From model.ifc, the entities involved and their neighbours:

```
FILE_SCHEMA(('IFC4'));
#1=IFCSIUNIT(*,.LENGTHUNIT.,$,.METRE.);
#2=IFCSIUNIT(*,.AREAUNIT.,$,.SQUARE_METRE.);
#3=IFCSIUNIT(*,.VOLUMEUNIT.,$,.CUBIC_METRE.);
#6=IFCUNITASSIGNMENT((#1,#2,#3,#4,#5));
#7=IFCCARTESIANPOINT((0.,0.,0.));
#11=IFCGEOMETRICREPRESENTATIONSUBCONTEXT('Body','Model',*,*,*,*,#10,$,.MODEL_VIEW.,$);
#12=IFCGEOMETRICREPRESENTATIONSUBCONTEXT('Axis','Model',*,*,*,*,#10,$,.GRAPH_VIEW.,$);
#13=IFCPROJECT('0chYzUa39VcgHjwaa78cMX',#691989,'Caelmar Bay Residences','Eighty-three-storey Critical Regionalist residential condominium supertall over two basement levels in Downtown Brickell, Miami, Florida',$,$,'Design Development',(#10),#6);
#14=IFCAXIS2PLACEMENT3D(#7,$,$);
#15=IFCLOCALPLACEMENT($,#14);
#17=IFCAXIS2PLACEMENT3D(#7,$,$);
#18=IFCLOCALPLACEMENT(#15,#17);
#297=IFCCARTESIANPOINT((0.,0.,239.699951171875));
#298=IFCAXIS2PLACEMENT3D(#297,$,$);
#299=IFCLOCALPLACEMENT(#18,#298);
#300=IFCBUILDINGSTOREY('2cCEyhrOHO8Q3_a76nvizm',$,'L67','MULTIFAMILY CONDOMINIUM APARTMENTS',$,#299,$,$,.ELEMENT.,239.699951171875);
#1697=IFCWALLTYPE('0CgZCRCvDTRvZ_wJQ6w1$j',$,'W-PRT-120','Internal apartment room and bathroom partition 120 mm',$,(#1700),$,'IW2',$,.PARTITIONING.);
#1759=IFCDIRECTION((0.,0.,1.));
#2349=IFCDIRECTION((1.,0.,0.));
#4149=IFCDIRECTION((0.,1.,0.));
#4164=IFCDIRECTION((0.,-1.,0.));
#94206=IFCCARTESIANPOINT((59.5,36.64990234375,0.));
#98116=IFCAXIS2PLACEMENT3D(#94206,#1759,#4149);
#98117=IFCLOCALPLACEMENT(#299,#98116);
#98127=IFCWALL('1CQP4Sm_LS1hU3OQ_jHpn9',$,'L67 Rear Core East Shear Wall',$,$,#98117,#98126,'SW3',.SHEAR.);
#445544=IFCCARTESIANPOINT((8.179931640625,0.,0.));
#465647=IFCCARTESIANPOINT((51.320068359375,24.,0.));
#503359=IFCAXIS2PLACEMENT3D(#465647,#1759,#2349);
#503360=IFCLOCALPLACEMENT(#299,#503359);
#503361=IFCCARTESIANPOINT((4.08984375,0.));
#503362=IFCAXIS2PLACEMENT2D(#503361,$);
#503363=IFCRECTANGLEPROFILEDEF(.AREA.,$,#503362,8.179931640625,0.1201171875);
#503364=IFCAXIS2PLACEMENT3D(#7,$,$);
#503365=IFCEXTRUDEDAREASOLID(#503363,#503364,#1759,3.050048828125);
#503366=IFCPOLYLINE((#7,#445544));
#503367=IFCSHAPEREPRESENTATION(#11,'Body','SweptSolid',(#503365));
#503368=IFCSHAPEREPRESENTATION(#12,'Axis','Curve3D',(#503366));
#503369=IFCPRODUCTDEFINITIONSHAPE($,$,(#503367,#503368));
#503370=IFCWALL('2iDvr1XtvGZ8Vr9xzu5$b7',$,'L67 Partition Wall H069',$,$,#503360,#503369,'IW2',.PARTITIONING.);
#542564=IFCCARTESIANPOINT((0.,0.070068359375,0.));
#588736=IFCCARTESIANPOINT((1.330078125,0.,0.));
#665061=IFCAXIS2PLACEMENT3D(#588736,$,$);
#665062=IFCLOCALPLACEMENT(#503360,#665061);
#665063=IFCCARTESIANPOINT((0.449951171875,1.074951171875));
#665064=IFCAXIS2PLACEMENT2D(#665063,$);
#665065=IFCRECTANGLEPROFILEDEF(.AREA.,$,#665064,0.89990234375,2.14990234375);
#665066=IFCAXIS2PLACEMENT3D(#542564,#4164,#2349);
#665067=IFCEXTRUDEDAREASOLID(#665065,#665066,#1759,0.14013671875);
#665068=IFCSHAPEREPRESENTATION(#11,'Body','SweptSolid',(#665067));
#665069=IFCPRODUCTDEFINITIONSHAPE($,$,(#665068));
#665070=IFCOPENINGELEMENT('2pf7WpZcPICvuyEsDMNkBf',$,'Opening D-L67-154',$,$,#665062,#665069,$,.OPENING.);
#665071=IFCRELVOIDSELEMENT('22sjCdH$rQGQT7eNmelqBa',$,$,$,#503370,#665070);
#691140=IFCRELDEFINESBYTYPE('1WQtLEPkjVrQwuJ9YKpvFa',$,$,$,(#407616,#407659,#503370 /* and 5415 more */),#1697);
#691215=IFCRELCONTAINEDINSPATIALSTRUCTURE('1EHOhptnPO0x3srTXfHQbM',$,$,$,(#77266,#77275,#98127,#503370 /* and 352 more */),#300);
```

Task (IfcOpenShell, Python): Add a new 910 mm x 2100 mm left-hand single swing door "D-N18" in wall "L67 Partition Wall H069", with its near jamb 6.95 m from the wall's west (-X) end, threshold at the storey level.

```python
import numpy as np
import ifcopenshell
import ifcopenshell.api.feature
import ifcopenshell.api.geometry
import ifcopenshell.api.root
import ifcopenshell.api.spatial
import ifcopenshell.geom
import ifcopenshell.util.element
import ifcopenshell.util.placement
import ifcopenshell.util.representation
import ifcopenshell.util.shape
import ifcopenshell.util.unit

model = ifcopenshell.open("model.ifc")
unit_scale = ifcopenshell.util.unit.calculate_unit_scale(model)
settings = ifcopenshell.geom.settings()


def volume(element):
    """Net volume in cubic metres, openings subtracted."""
    shape = ifcopenshell.geom.create_shape(settings, element)
    return ifcopenshell.util.shape.get_volume(shape.geometry)


wall = model.by_id(503370)
storey = ifcopenshell.util.element.get_container(wall, ifc_class="IfcBuildingStorey")
context = ifcopenshell.util.representation.get_context(model, "Model", "Body", "MODEL_VIEW")
before = volume(wall)

width, height, from_end, sill = 0.91, 2.1, 6.95, 0.0  # metres

# The wall runs along its own X axis, and the end named is its -X end.
wall_shape = ifcopenshell.geom.create_shape(settings, wall)
x, y, z = ifcopenshell.util.shape.get_vertices(wall_shape.geometry).T
start = x.min() + from_end
face, thickness = float(y.min()), float(y.max() - y.min())
wall_matrix = ifcopenshell.util.placement.get_local_placement(wall.ObjectPlacement)
level = ifcopenshell.util.placement.get_local_placement(storey.ObjectPlacement)[2, 3]


def in_wall(x, y):
    """Placement at x, y metres in the wall's axes, at sill height."""
    matrix = wall_matrix.copy()
    matrix[:, 3] = wall_matrix @ np.array([x / unit_scale, y / unit_scale, 0.0, 1.0])
    matrix[2, 3] = level + sill / unit_scale
    return matrix


# Opening: a box that overshoots both wall faces by 50 mm.
opening = ifcopenshell.api.root.create_entity(model, ifc_class="IfcOpeningElement", predefined_type="OPENING")
box = ifcopenshell.api.geometry.add_wall_representation(
    model, context=context, length=width, height=height, thickness=thickness + 0.1
)
ifcopenshell.api.geometry.assign_representation(model, product=opening, representation=box)
ifcopenshell.api.geometry.edit_object_placement(model, product=opening, matrix=in_wall(start, face - 0.05), is_si=False)
ifcopenshell.api.feature.add_feature(model, feature=opening, element=wall)

door = ifcopenshell.api.root.create_entity(model, ifc_class="IfcDoor", name="D-N18", predefined_type="DOOR")
door.OverallWidth, door.OverallHeight = width / unit_scale, height / unit_scale
door.OperationType = "SINGLE_SWING_LEFT"
body = ifcopenshell.api.geometry.add_door_representation(
    model,
    context=context,
    overall_width=door.OverallWidth,
    overall_height=door.OverallHeight,
    operation_type="SINGLE_SWING_LEFT",
    lining_properties={"LiningDepth": thickness / unit_scale, "ThresholdDepth": thickness / unit_scale},
)
ifcopenshell.api.geometry.assign_representation(model, product=door, representation=body)
ifcopenshell.api.spatial.assign_container(model, products=[door], relating_structure=storey)
ifcopenshell.api.feature.add_filling(model, opening=opening, element=door)

# The lining spans the wall, so the door starts at the wall face.
ifcopenshell.api.geometry.edit_object_placement(model, product=door, matrix=in_wall(start, face), is_si=False)

after = volume(wall)

print(f"wall volume {before:.3f} -> {after:.3f} m3")

model.write("model_v2.ifc")
```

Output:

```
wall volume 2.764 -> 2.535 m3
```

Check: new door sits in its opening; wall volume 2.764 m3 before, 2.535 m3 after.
